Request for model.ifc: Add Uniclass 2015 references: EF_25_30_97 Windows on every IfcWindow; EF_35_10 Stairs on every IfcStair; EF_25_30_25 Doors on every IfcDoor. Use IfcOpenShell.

First a look at what the model holds.

```python
import ifcopenshell

model = ifcopenshell.open("model.ifc")
print(model.schema)
print("classifications:", [c.Name for c in model.by_type("IfcClassification")])
for ifc_class in ("IfcDoor", "IfcRoof", "IfcStair", "IfcWall", "IfcWindow"):
    print(ifc_class, len(model.by_type(ifc_class)))
```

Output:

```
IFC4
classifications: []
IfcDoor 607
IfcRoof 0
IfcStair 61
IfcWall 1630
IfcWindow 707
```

```python
import ifcopenshell
import ifcopenshell.api.classification

model = ifcopenshell.open("model.ifc")

system = ifcopenshell.api.classification.add_classification(model, classification="Uniclass 2015")

codes = {
    "IfcWindow": ("EF_25_30_97", "Windows"),
    "IfcStair": ("EF_35_10", "Stairs"),
    "IfcDoor": ("EF_25_30_25", "Doors"),
}
for ifc_class, (code, name) in codes.items():
    products = model.by_type(ifc_class)
    ifcopenshell.api.classification.add_reference(
        model, products=products, classification=system, identification=code, name=name
    )
    print(code, len(products))

model.write("model_rev.ifc")
```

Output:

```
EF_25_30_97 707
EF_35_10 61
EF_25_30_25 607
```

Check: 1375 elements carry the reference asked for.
